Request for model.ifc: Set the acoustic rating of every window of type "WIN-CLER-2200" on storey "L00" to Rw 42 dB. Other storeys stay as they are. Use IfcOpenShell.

First a look at what the model holds.

```python
import ifcopenshell
import ifcopenshell.util.element

model = ifcopenshell.open("model.ifc")
print(model.schema)
storey = next(s for s in model.by_type("IfcBuildingStorey") if s.Name == "L00")
windows = [e for e in ifcopenshell.util.element.get_decomposition(storey) if e.is_a("IfcWindow")]
seen = {}
for e in windows:
    element_type = ifcopenshell.util.element.get_type(e)
    key = (element_type.Name if element_type != e and element_type else None, ifcopenshell.util.element.get_pset(e, "Pset_WindowCommon", "AcousticRating"))
    seen[key] = seen.get(key, 0) + 1
for (name, value), count in sorted(seen.items(), key=str):
    print(count, "x", name, "|", value)
```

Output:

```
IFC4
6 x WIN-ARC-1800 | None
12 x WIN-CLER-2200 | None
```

```python
import ifcopenshell
import ifcopenshell.api.pset
import ifcopenshell.util.element

model = ifcopenshell.open("model.ifc")

storey = next(s for s in model.by_type("IfcBuildingStorey") if s.Name == "L00")
windows = [e for e in ifcopenshell.util.element.get_decomposition(storey) if e.is_a("IfcWindow")]

count = 0
for e in windows:
    element_type = ifcopenshell.util.element.get_type(e)
    if element_type in (None, e) or element_type.Name != "WIN-CLER-2200":
        continue
    # add_pset returns the element's existing set when there is one.
    pset = ifcopenshell.api.pset.add_pset(model, product=e, name="Pset_WindowCommon")
    ifcopenshell.api.pset.edit_pset(model, pset=pset, properties={"AcousticRating": "Rw 42 dB"})
    count += 1

print(count, "windows updated")

model.write("model_rev.ifc")
```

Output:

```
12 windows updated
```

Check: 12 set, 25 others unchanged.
